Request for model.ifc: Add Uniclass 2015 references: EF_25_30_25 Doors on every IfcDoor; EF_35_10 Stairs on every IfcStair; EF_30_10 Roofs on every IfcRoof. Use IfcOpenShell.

First a look at what the model holds.

```python
import ifcopenshell

model = ifcopenshell.open("model.ifc")
print(model.schema)
print("classifications:", [c.Name for c in model.by_type("IfcClassification")])
for ifc_class in ("IfcDoor", "IfcRoof", "IfcStair", "IfcWall", "IfcWindow"):
    print(ifc_class, len(model.by_type(ifc_class)))
```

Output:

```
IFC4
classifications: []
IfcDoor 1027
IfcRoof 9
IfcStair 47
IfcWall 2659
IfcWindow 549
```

```python
import ifcopenshell
import ifcopenshell.api.classification

model = ifcopenshell.open("model.ifc")

system = ifcopenshell.api.classification.add_classification(model, classification="Uniclass 2015")

codes = {
    "IfcDoor": ("EF_25_30_25", "Doors"),
    "IfcStair": ("EF_35_10", "Stairs"),
    "IfcRoof": ("EF_30_10", "Roofs"),
}
for ifc_class, (code, name) in codes.items():
    products = model.by_type(ifc_class)
    ifcopenshell.api.classification.add_reference(
        model, products=products, classification=system, identification=code, name=name
    )
    print(code, len(products))

model.write("model-out.ifc")
```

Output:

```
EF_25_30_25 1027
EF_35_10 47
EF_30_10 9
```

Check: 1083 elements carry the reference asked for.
